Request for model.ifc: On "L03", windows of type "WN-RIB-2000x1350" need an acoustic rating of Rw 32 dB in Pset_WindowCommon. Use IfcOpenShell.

First a look at what the model holds.

```python
import ifcopenshell
import ifcopenshell.util.element

model = ifcopenshell.open("model.ifc")
print(model.schema)
storey = next(s for s in model.by_type("IfcBuildingStorey") if s.Name == "L03")
windows = [e for e in ifcopenshell.util.element.get_decomposition(storey) if e.is_a("IfcWindow")]
seen = {}
for e in windows:
    element_type = ifcopenshell.util.element.get_type(e)
    key = (element_type.Name if element_type != e and element_type else None, ifcopenshell.util.element.get_pset(e, "Pset_WindowCommon", "AcousticRating"))
    seen[key] = seen.get(key, 0) + 1
for (name, value), count in sorted(seen.items(), key=str):
    print(count, "x", name, "|", value)
```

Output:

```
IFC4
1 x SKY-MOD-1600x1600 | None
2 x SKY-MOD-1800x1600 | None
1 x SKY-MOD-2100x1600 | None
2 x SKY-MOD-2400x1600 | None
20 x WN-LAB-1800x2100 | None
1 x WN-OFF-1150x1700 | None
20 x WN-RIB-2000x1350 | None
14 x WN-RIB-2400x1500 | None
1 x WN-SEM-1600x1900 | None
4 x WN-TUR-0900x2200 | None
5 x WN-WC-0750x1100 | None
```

```python
import ifcopenshell
import ifcopenshell.api.pset
import ifcopenshell.util.element

model = ifcopenshell.open("model.ifc")

storey = next(s for s in model.by_type("IfcBuildingStorey") if s.Name == "L03")
windows = [e for e in ifcopenshell.util.element.get_decomposition(storey) if e.is_a("IfcWindow")]

count = 0
for e in windows:
    element_type = ifcopenshell.util.element.get_type(e)
    if element_type in (None, e) or element_type.Name != "WN-RIB-2000x1350":
        continue
    # add_pset returns the element's existing set when there is one.
    pset = ifcopenshell.api.pset.add_pset(model, product=e, name="Pset_WindowCommon")
    ifcopenshell.api.pset.edit_pset(model, pset=pset, properties={"AcousticRating": "Rw 32 dB"})
    count += 1

print(count, "windows updated")

model.write("model_edited.ifc")
```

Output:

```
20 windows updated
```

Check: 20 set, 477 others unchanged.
